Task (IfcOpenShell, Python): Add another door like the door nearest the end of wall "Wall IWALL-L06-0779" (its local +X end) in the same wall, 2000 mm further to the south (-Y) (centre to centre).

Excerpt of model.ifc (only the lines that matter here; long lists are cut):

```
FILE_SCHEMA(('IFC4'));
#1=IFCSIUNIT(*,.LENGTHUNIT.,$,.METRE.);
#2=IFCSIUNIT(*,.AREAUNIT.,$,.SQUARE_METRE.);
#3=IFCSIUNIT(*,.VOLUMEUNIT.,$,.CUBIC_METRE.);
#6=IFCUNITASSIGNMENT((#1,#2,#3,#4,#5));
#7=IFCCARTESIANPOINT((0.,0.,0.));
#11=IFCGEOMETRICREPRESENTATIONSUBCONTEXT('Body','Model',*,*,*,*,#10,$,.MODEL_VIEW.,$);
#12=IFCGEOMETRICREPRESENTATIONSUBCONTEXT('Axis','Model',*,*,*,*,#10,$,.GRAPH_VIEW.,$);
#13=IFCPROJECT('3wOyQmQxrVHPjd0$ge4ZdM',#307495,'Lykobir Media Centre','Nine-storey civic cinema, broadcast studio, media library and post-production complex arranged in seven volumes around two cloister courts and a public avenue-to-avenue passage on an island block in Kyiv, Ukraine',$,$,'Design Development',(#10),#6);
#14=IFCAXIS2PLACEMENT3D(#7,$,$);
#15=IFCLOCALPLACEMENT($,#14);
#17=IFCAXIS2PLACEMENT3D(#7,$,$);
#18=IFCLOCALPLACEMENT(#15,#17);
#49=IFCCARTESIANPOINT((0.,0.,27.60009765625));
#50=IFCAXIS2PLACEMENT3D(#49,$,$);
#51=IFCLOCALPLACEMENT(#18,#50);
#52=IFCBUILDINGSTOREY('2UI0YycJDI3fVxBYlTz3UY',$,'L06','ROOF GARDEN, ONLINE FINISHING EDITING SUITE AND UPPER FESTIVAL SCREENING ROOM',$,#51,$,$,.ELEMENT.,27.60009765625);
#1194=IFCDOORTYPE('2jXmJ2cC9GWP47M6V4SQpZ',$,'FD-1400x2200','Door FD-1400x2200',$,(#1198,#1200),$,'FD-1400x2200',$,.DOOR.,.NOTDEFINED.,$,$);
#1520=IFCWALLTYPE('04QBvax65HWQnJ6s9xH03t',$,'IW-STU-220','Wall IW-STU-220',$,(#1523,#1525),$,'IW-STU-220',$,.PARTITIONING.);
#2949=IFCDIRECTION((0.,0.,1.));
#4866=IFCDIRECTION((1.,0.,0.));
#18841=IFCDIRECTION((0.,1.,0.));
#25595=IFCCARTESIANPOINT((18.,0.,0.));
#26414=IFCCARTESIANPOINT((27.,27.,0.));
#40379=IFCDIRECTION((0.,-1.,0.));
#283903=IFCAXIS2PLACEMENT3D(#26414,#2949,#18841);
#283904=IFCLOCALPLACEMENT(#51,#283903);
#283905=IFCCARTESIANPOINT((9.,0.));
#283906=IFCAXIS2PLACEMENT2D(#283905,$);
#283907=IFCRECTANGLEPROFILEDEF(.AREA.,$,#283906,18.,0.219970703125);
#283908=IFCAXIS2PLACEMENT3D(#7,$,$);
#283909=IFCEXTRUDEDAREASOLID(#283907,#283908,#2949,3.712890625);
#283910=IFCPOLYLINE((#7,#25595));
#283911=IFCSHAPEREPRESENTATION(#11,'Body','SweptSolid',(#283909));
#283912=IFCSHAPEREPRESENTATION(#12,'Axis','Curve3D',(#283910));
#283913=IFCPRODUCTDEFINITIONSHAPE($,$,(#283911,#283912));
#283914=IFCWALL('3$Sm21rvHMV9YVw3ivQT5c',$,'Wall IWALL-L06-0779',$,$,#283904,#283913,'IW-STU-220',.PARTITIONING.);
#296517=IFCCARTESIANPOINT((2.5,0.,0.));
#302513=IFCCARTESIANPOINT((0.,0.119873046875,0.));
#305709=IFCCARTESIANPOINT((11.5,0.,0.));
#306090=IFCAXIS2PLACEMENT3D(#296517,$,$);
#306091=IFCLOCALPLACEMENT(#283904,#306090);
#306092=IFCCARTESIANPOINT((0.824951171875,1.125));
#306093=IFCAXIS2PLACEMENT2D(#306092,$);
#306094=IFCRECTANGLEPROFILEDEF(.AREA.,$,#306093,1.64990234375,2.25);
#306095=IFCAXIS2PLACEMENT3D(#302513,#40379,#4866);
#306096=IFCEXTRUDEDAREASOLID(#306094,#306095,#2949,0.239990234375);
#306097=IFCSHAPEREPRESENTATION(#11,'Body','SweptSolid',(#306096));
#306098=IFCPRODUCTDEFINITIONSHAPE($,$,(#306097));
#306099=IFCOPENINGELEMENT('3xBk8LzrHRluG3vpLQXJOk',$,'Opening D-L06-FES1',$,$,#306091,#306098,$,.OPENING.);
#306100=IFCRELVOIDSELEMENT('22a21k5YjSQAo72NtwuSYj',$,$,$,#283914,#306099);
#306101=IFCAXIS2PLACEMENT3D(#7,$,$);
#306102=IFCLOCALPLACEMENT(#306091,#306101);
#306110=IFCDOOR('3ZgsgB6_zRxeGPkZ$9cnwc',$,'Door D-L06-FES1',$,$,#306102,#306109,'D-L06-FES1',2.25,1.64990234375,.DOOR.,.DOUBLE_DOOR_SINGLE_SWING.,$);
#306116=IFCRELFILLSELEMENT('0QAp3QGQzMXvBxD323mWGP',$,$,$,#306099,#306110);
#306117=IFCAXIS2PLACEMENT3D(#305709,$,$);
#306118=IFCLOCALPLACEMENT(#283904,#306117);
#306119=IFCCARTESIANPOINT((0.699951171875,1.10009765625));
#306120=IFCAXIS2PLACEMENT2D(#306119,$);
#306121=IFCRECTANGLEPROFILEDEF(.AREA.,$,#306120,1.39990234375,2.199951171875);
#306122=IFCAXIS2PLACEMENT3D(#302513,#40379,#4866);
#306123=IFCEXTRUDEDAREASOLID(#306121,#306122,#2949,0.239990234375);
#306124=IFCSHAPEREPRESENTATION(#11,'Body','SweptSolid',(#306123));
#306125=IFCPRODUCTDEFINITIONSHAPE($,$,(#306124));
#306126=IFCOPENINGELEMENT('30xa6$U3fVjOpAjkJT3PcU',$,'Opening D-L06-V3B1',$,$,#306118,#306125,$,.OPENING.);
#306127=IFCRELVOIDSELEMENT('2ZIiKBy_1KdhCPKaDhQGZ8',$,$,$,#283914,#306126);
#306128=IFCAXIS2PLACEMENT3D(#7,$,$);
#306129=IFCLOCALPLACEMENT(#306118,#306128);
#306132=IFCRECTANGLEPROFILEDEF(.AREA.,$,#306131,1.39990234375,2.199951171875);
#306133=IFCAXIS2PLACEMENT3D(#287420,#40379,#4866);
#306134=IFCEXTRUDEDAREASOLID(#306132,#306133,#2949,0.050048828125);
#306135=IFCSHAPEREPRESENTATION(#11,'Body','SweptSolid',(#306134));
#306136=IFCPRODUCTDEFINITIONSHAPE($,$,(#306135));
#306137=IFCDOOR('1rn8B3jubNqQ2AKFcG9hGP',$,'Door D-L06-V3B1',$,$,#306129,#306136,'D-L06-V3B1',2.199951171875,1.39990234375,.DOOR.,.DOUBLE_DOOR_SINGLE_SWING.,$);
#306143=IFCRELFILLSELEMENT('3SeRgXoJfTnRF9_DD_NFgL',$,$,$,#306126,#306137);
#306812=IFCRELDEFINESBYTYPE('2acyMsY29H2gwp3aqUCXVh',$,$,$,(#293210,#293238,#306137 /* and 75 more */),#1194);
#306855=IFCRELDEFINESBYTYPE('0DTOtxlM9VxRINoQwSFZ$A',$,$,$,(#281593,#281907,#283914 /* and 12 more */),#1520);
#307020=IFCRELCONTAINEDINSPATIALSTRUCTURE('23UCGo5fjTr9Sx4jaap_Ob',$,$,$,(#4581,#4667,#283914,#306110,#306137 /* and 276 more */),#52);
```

```python
import ifcopenshell
import ifcopenshell.api.feature
import ifcopenshell.api.geometry
import ifcopenshell.api.root
import ifcopenshell.geom
import ifcopenshell.util.element
import ifcopenshell.util.placement
import ifcopenshell.util.shape

model = ifcopenshell.open("model.ifc")
settings = ifcopenshell.geom.settings()


def volume(element):
    """Net volume in cubic metres, openings subtracted."""
    shape = ifcopenshell.geom.create_shape(settings, element)
    return ifcopenshell.util.shape.get_volume(shape.geometry)


door = model.by_guid("1rn8B3jubNqQ2AKFcG9hGP")
opening = door.FillsVoids[0].RelatingOpeningElement
wall = opening.VoidsElements[0].RelatingBuildingElement
before = volume(wall)
shift = ifcopenshell.util.placement.get_local_placement(wall.ObjectPlacement)[:3, 0] * -2.0

# copy_class copies the void relationship, type, container and properties, but no geometry.
new_opening = ifcopenshell.api.root.copy_class(model, product=opening)
new_opening.Representation = ifcopenshell.util.element.copy_deep(
    model, opening.Representation, exclude=["IfcGeometricRepresentationContext", "IfcRepresentationMap"]
)
new_door = ifcopenshell.api.root.copy_class(model, product=door)
new_door.Representation = ifcopenshell.util.element.copy_deep(
    model, door.Representation, exclude=["IfcGeometricRepresentationContext", "IfcRepresentationMap"]
)
new_door.Tag = None
ifcopenshell.api.feature.add_filling(model, opening=new_opening, element=new_door)

for old, new in ((opening, new_opening), (door, new_door)):
    matrix = ifcopenshell.util.placement.get_local_placement(old.ObjectPlacement)
    matrix[:3, 3] += shift
    ifcopenshell.api.geometry.edit_object_placement(model, product=new, matrix=matrix, is_si=False)

after = volume(wall)

print(f"wall volume {before:.3f} -> {after:.3f} m3")

model.write("model_v2.ifc")
```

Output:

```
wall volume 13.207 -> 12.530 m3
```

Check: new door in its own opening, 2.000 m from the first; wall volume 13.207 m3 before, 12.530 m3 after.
